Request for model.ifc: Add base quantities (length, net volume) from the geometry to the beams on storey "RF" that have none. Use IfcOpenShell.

First a look at what the model holds.

```python
import ifcopenshell
import ifcopenshell.util.element
import ifcopenshell.util.unit

model = ifcopenshell.open("model.ifc")
print(model.schema)
for unit_type in ("LENGTHUNIT", "AREAUNIT", "VOLUMEUNIT"):
    print(unit_type, ifcopenshell.util.unit.calculate_unit_scale(model, unit_type))
storey = next(s for s in model.by_type("IfcBuildingStorey") if s.Name == "RF")
beams = [e for e in ifcopenshell.util.element.get_decomposition(storey) if e.is_a("IfcBeam")]
for e in sorted(beams, key=lambda e: e.id()):
    print(e.id(), e.is_a(), e.Name, list(ifcopenshell.util.element.get_psets(e, qtos_only=True)), sep=" | ")
```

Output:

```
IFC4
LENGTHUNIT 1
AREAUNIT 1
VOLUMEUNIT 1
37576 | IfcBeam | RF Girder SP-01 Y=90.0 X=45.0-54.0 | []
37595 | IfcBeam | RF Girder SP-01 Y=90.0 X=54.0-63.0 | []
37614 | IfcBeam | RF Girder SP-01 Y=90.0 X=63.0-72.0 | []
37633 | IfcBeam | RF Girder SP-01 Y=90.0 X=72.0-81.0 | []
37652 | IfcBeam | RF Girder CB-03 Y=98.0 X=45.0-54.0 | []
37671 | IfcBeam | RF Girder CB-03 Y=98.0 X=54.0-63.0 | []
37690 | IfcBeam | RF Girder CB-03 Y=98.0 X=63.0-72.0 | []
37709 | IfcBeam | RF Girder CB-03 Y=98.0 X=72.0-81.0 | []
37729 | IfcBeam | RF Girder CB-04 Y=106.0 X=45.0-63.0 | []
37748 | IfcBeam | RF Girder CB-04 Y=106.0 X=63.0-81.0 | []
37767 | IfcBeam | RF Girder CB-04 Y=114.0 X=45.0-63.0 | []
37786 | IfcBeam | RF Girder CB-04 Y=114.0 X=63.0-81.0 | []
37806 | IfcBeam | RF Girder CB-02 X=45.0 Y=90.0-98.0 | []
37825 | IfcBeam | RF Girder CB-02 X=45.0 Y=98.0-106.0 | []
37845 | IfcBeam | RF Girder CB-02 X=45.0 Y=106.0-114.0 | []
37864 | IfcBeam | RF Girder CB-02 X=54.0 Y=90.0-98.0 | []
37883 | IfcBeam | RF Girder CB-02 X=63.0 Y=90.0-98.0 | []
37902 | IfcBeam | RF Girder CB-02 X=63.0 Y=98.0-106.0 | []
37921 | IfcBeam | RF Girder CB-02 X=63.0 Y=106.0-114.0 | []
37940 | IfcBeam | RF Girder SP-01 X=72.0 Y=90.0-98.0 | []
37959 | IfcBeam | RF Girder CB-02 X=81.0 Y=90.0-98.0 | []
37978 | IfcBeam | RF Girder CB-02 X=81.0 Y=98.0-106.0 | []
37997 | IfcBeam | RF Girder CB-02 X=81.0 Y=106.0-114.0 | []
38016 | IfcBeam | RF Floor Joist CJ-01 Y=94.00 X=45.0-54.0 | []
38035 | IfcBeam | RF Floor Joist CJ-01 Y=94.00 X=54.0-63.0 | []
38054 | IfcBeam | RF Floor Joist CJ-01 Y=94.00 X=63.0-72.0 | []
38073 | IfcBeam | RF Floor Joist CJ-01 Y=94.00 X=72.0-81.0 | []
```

```python
import ifcopenshell
import ifcopenshell.api.pset
import ifcopenshell.geom
import ifcopenshell.util.element
import ifcopenshell.util.shape
import ifcopenshell.util.unit

model = ifcopenshell.open("model.ifc")
unit_scale = ifcopenshell.util.unit.calculate_unit_scale(model)
volume_scale = ifcopenshell.util.unit.calculate_unit_scale(model, "VOLUMEUNIT")
settings = ifcopenshell.geom.settings()

storey = next(s for s in model.by_type("IfcBuildingStorey") if s.Name == "RF")
beams = [e for e in ifcopenshell.util.element.get_decomposition(storey) if e.is_a("IfcBeam")]

for e in sorted(beams, key=lambda e: e.id()):
    if ifcopenshell.util.element.get_psets(e, qtos_only=True, should_inherit=False):
        continue
    # Geometry comes back in metres, in the element's own axes.
    shape = ifcopenshell.geom.create_shape(settings, e)
    values = {
        "Length": ifcopenshell.util.shape.get_max_xyz(shape.geometry) / unit_scale,
        "NetVolume": ifcopenshell.util.shape.get_volume(shape.geometry) / volume_scale,
    }
    qto = ifcopenshell.api.pset.add_qto(model, product=e, name="Qto_BeamBaseQuantities")
    ifcopenshell.api.pset.edit_qto(model, qto=qto, properties=values)
    print(e.id(), {k: round(v, 3) for k, v in values.items()})

model.write("model_updated.ifc")
```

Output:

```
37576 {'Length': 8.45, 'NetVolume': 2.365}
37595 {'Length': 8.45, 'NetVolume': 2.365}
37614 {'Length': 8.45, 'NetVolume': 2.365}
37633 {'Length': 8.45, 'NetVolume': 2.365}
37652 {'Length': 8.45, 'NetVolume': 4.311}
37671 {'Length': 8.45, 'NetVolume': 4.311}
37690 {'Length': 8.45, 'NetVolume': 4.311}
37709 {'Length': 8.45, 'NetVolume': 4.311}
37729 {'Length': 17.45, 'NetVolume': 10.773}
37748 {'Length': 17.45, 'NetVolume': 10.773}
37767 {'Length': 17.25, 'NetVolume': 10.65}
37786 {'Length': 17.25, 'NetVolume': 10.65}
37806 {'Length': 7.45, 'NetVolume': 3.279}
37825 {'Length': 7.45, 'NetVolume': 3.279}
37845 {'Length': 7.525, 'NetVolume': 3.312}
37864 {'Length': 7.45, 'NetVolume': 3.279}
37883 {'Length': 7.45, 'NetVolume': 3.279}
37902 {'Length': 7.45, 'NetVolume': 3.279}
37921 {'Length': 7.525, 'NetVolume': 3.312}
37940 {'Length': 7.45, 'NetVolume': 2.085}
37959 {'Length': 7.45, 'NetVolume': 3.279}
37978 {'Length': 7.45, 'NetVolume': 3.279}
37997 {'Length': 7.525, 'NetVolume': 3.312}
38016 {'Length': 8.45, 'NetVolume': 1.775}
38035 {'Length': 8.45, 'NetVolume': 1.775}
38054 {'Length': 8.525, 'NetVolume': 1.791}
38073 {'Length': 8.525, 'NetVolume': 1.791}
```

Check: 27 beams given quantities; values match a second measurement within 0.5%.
